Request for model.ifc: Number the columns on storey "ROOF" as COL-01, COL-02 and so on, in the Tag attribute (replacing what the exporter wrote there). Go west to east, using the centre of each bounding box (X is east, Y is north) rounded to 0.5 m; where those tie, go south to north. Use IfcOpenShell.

First a look at what the model holds.

```python
import ifcopenshell
import ifcopenshell.util.element
import ifcopenshell.util.placement

model = ifcopenshell.open("model.ifc")
print(model.schema)
storey = next(s for s in model.by_type("IfcBuildingStorey") if s.Name == "ROOF")
columns = [e for e in ifcopenshell.util.element.get_decomposition(storey) if e.is_a("IfcColumn")]
for e in sorted(columns, key=lambda e: e.id()):
    origin = ifcopenshell.util.placement.get_local_placement(e.ObjectPlacement)[:3, 3]
    print(e.id(), e.Tag, e.Name, origin.round(2) + 0.0, sep=" | ")
```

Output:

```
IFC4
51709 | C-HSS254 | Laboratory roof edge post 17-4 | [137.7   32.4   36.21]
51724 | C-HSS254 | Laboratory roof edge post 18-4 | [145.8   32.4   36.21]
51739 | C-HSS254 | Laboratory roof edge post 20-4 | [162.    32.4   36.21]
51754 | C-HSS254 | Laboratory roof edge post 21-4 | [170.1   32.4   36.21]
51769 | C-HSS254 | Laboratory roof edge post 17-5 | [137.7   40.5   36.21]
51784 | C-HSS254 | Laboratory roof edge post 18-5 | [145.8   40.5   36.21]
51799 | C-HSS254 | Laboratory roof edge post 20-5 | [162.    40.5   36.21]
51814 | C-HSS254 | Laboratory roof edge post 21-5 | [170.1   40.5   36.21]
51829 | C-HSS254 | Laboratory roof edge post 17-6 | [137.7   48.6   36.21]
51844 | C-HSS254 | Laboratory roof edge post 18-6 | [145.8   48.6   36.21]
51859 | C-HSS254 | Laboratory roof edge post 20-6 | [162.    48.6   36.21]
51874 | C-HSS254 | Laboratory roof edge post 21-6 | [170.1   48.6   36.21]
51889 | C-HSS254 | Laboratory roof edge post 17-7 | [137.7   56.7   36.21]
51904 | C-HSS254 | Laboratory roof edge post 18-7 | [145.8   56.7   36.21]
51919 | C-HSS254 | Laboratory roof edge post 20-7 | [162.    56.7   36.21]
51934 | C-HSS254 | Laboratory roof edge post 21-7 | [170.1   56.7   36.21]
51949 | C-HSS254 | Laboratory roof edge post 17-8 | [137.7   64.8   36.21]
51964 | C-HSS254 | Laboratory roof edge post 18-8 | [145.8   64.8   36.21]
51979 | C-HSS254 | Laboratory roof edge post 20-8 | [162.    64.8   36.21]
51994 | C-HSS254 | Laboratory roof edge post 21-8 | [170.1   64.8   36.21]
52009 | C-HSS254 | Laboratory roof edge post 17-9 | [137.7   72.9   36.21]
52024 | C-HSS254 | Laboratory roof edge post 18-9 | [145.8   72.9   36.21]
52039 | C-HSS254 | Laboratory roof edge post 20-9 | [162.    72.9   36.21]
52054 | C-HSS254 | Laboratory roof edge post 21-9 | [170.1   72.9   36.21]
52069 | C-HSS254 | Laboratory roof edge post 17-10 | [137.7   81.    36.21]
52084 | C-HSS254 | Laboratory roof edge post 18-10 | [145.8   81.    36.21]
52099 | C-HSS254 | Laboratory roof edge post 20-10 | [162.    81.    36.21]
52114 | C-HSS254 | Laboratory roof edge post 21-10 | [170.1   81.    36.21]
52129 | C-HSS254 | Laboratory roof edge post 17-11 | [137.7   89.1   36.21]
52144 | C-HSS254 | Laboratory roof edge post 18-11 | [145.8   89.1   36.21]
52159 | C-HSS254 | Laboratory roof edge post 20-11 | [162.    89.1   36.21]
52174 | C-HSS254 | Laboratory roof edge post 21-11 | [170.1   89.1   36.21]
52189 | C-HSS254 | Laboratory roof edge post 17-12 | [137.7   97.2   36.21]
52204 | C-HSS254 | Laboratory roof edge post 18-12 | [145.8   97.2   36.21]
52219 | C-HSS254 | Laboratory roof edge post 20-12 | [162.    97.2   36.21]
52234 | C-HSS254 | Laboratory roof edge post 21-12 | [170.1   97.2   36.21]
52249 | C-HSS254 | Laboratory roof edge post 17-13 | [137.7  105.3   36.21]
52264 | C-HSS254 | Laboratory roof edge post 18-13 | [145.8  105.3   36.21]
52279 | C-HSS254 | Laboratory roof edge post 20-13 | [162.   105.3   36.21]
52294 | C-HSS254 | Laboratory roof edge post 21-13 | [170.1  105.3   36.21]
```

```python
import ifcopenshell
import ifcopenshell.geom
import ifcopenshell.util.element
import ifcopenshell.util.shape

model = ifcopenshell.open("model.ifc")
settings = ifcopenshell.geom.settings()
settings.set("use-world-coords", True)


def centre(element):
    shape = ifcopenshell.geom.create_shape(settings, element)
    return ifcopenshell.util.shape.get_bbox_centroid(shape.geometry)


storey = next(s for s in model.by_type("IfcBuildingStorey") if s.Name == "ROOF")
columns = [e for e in ifcopenshell.util.element.get_decomposition(storey) if e.is_a("IfcColumn")]

# Insertion points can sit at a corner or the storey origin, so sort by the geometry (in metres).
centres = {e: centre(e) for e in columns}
columns.sort(key=lambda e: (round(centres[e][0] / 0.5), centres[e][1]))

for i, e in enumerate(columns, start=1):
    number = f"COL-{i:02d}"
    e.Tag = number
    print(e.id(), number)

model.write("model_rev.ifc")
```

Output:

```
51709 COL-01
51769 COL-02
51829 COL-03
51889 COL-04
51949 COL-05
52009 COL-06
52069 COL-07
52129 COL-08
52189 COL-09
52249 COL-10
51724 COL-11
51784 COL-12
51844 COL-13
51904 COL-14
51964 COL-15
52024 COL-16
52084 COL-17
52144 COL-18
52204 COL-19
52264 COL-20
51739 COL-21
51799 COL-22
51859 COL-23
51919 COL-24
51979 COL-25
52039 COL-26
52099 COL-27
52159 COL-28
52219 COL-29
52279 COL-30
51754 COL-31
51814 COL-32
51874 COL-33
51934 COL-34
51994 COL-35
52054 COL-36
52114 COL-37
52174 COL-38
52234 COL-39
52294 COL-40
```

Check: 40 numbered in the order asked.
